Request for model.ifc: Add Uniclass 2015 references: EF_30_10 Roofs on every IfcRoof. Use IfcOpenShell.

First a look at what the model holds.

```python
import ifcopenshell

model = ifcopenshell.open("model.ifc")
print(model.schema)
print("classifications:", [c.Name for c in model.by_type("IfcClassification")])
for ifc_class in ("IfcDoor", "IfcRoof", "IfcStair", "IfcWall", "IfcWindow"):
    print(ifc_class, len(model.by_type(ifc_class)))
```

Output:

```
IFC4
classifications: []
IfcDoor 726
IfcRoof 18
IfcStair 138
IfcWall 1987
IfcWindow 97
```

```python
import ifcopenshell
import ifcopenshell.api.classification

model = ifcopenshell.open("model.ifc")

system = ifcopenshell.api.classification.add_classification(model, classification="Uniclass 2015")

codes = {
    "IfcRoof": ("EF_30_10", "Roofs"),
}
for ifc_class, (code, name) in codes.items():
    products = model.by_type(ifc_class)
    ifcopenshell.api.classification.add_reference(
        model, products=products, classification=system, identification=code, name=name
    )
    print(code, len(products))

model.write("model_rev.ifc")
```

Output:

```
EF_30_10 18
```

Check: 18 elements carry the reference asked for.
